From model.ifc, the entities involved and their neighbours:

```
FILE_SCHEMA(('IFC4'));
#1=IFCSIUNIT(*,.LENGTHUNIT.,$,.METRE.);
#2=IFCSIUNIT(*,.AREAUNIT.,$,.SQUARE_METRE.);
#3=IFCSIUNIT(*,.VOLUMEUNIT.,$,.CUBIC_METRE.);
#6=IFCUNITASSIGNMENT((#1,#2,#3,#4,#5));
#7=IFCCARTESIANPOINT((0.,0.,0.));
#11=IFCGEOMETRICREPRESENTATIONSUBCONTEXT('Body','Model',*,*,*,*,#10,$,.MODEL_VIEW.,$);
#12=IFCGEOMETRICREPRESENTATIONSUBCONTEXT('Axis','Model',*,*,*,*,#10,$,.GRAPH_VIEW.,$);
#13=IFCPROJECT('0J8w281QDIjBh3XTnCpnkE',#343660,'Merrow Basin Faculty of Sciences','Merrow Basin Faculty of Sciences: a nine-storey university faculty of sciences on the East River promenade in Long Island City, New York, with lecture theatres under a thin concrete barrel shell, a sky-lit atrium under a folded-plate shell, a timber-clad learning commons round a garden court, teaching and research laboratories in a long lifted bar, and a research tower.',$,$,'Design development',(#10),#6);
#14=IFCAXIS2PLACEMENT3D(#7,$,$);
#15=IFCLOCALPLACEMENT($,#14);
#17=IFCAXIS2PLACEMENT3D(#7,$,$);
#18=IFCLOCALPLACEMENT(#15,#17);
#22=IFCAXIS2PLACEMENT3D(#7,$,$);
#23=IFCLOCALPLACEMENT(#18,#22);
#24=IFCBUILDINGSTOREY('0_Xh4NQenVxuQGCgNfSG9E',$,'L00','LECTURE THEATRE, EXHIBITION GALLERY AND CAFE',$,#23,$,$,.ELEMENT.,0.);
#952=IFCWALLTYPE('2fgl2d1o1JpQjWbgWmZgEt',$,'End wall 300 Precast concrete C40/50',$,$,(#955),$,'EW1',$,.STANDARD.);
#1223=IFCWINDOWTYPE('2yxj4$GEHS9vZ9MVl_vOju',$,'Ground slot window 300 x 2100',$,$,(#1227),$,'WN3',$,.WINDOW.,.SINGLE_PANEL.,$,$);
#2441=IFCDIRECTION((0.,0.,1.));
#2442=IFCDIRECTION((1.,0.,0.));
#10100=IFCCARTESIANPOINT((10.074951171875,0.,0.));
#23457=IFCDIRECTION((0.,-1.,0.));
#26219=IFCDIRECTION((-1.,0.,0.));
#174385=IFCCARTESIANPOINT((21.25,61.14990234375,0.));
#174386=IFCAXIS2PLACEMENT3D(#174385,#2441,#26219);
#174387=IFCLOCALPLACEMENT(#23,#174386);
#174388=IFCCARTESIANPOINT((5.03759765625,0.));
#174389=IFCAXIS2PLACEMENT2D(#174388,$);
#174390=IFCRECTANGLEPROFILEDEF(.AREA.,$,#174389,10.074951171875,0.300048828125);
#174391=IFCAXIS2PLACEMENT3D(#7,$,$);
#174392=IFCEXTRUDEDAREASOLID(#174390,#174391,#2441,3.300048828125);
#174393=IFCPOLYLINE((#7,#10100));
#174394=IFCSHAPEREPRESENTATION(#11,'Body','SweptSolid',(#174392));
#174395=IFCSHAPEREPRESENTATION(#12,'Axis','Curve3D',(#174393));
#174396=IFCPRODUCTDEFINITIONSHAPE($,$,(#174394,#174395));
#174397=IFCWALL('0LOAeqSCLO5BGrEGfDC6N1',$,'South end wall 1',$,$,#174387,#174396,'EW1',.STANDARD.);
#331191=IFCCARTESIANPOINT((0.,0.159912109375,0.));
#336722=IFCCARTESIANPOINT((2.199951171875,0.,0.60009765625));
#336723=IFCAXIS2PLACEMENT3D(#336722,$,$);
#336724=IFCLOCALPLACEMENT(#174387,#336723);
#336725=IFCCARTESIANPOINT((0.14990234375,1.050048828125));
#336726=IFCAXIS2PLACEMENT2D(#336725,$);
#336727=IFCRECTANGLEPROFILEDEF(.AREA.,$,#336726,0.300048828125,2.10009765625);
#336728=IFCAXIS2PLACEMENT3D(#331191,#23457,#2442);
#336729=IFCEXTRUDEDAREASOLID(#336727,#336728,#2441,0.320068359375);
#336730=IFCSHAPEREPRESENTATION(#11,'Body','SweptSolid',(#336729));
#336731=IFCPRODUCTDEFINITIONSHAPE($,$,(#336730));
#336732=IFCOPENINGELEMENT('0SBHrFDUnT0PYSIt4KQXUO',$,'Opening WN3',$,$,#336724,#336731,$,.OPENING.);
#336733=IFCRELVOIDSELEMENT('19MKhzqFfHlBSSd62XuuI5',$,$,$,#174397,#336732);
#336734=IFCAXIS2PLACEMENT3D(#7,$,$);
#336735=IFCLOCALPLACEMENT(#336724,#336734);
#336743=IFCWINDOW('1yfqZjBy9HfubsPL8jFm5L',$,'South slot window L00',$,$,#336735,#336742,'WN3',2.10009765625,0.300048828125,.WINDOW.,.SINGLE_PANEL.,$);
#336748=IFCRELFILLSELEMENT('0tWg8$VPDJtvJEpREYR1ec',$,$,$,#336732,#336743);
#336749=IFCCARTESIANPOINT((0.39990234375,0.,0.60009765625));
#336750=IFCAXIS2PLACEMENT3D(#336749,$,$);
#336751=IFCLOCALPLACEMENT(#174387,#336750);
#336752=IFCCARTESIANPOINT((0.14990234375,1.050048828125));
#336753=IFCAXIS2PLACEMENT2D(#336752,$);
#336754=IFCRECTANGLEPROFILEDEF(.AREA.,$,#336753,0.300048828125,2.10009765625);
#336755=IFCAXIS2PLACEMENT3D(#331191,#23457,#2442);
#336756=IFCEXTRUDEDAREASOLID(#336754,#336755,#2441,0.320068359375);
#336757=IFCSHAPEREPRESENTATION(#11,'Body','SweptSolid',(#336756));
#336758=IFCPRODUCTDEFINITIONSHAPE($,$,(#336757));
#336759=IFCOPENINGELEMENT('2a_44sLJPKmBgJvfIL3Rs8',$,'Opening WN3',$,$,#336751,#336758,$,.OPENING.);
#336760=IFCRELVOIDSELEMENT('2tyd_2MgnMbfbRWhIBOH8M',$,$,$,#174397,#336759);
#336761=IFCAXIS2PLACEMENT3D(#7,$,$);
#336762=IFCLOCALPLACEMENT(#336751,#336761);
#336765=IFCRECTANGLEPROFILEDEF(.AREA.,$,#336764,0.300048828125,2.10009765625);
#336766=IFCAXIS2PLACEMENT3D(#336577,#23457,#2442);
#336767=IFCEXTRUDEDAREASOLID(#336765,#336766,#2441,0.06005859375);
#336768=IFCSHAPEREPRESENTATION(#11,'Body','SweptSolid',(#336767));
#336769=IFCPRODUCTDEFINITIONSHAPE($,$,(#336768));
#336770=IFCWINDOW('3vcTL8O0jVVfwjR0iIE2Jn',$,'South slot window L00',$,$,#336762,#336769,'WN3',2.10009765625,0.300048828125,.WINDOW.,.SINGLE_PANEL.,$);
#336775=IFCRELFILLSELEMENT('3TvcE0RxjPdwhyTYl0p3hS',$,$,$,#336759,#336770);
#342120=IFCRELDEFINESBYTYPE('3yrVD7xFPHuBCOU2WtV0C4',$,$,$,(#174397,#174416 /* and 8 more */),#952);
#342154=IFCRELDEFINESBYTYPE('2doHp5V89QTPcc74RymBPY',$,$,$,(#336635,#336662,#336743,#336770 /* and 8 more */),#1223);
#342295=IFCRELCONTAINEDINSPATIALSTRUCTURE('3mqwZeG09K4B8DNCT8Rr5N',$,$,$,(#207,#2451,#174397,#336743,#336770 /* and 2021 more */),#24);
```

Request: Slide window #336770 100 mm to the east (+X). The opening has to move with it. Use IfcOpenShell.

```python
import ifcopenshell
import ifcopenshell.api.geometry
import ifcopenshell.util.placement
import ifcopenshell.util.unit

model = ifcopenshell.open("model.ifc")
unit_scale = ifcopenshell.util.unit.calculate_unit_scale(model)

window = model.by_id(336770)
opening = window.FillsVoids[0].RelatingOpeningElement
wall = opening.VoidsElements[0].RelatingBuildingElement

wall_matrix = ifcopenshell.util.placement.get_local_placement(wall.ObjectPlacement)
shift = wall_matrix[:3, 0] * -0.1 / unit_scale
before = ifcopenshell.util.placement.get_local_placement(window.ObjectPlacement)[:3, 3].copy()

# The window is placed relative to its opening, so it follows when the opening moves.
matrix = ifcopenshell.util.placement.get_local_placement(opening.ObjectPlacement)
matrix[:3, 3] += shift
ifcopenshell.api.geometry.edit_object_placement(
    model, product=opening, matrix=matrix, is_si=False, should_transform_children=True
)

after = ifcopenshell.util.placement.get_local_placement(window.ObjectPlacement)[:3, 3]
print("window moved by", (after - before).round(3) + 0.0)

model.write("model_v2.ifc")
```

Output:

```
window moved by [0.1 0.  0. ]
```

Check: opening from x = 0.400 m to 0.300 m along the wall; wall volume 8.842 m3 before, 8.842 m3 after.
